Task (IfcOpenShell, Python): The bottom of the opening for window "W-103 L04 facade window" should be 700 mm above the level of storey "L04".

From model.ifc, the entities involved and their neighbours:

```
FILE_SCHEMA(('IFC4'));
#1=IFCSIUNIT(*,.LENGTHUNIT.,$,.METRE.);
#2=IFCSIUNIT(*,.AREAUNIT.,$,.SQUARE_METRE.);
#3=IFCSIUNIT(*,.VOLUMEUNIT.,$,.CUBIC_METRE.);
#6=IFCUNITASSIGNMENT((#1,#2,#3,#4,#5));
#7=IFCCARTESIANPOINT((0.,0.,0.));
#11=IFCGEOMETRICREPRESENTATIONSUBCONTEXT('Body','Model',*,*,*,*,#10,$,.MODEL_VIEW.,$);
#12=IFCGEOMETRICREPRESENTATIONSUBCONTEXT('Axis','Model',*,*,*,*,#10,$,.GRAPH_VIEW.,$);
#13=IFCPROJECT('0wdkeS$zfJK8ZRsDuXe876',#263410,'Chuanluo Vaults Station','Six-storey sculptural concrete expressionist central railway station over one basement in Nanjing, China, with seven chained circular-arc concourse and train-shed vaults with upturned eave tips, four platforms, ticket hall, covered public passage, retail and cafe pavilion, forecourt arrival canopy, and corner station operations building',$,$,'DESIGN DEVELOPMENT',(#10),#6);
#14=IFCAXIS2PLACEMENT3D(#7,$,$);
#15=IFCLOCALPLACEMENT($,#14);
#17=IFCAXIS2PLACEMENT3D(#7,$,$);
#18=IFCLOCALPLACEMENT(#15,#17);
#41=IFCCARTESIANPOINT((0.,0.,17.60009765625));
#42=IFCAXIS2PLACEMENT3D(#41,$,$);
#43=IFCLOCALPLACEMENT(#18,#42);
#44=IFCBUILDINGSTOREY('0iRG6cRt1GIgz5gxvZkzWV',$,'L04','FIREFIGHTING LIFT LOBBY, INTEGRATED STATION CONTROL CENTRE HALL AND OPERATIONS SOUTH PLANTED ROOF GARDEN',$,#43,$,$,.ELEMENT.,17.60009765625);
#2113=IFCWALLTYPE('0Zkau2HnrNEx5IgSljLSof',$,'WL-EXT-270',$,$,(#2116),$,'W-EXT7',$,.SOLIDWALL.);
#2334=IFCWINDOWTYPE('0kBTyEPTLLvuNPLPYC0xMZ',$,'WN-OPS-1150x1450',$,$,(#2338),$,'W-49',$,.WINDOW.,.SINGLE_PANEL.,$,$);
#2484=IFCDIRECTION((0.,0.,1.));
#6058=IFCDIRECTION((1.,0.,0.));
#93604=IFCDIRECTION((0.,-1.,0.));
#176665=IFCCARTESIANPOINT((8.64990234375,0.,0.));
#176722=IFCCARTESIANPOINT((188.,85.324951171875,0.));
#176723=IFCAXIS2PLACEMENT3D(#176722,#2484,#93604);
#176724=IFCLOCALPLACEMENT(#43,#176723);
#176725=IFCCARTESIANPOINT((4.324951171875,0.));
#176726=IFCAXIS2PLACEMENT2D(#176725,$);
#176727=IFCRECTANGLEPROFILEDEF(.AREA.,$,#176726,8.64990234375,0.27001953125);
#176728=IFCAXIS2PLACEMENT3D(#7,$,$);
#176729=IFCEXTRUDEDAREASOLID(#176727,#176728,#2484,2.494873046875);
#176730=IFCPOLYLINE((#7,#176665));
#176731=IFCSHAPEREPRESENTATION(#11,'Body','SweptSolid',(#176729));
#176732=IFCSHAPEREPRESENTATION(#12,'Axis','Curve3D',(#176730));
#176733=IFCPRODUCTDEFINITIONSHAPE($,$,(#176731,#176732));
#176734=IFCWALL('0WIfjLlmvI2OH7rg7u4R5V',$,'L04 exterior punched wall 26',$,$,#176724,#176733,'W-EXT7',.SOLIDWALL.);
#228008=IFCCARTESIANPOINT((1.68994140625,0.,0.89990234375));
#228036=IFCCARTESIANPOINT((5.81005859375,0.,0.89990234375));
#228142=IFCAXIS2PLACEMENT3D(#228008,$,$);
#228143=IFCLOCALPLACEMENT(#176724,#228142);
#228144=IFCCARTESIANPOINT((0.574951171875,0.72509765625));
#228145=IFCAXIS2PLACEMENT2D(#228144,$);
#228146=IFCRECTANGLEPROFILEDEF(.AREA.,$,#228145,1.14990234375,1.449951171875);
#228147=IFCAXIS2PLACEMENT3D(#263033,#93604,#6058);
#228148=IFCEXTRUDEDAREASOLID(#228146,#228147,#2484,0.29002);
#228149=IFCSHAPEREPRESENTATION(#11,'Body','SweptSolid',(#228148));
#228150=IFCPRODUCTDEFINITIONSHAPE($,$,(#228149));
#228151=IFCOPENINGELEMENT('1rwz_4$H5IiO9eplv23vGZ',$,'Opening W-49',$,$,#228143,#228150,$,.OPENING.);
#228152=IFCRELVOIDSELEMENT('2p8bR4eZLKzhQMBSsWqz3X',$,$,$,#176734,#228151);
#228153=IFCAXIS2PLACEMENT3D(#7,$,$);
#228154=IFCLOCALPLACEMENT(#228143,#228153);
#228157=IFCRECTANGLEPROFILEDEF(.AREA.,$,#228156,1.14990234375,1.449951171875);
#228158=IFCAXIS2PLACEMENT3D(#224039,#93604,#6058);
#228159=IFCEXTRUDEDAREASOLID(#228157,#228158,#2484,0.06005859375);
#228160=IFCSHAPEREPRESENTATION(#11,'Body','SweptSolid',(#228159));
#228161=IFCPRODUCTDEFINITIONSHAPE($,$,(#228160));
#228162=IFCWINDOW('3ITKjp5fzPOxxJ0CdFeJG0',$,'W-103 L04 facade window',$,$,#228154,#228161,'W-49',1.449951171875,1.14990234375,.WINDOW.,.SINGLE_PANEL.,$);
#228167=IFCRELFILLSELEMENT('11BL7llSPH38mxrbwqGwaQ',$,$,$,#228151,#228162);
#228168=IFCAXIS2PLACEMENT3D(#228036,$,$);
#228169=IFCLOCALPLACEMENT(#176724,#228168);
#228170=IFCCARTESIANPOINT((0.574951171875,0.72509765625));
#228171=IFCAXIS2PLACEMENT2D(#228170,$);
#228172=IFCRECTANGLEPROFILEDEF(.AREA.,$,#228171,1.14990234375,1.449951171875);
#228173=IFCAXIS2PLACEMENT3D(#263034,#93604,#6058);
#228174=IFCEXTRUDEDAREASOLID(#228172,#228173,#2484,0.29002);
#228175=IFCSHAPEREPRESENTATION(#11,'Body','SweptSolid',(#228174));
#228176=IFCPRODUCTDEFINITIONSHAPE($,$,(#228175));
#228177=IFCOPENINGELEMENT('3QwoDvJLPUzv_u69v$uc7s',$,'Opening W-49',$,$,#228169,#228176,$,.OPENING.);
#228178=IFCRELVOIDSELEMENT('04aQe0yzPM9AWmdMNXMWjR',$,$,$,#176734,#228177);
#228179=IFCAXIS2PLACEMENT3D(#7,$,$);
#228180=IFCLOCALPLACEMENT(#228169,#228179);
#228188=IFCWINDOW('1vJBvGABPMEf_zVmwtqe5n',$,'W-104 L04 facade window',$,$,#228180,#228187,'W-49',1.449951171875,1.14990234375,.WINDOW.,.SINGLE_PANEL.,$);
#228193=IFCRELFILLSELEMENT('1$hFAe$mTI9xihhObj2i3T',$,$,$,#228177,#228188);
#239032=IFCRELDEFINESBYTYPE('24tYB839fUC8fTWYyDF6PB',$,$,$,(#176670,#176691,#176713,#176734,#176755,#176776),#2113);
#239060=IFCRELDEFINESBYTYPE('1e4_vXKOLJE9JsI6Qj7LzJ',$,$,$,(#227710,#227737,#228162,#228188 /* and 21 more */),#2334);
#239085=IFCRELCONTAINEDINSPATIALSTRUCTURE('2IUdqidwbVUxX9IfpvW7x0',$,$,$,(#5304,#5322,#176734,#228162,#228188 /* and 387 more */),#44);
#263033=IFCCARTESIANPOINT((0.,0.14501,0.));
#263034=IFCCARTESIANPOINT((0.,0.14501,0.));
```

```python
import numpy as np
import ifcopenshell
import ifcopenshell.api.geometry
import ifcopenshell.geom
import ifcopenshell.util.element
import ifcopenshell.util.placement
import ifcopenshell.util.shape
import ifcopenshell.util.unit

model = ifcopenshell.open("model.ifc")
unit_scale = ifcopenshell.util.unit.calculate_unit_scale(model)

window = model.by_id(228162)
opening = window.FillsVoids[0].RelatingOpeningElement
storey = ifcopenshell.util.element.get_container(window, ifc_class="IfcBuildingStorey")
level = ifcopenshell.util.placement.get_local_placement(storey.ObjectPlacement)[2, 3]

# The opening's origin need not be at the sill, so measure its lowest point.
shape = ifcopenshell.geom.create_shape(ifcopenshell.geom.settings(), opening)
bottom = ifcopenshell.util.shape.get_shape_bottom_elevation(shape, shape.geometry) / unit_scale
dz = level + 0.7 / unit_scale - bottom

shift = np.array([0.0, 0.0, dz])
# The window is placed relative to its opening, so it follows when the opening moves.
matrix = ifcopenshell.util.placement.get_local_placement(opening.ObjectPlacement)
matrix[:3, 3] += shift
ifcopenshell.api.geometry.edit_object_placement(
    model, product=opening, matrix=matrix, is_si=False, should_transform_children=True
)

print(f"moved by {dz * unit_scale:+.3f} m")

model.write("model-out.ifc")
```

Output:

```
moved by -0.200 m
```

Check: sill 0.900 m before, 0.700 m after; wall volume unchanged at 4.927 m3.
